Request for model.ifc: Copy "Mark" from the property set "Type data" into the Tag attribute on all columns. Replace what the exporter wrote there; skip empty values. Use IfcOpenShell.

First a look at what the model holds.

```python
import ifcopenshell
import ifcopenshell.util.element

model = ifcopenshell.open("model.ifc")
print(model.schema)
columns = model.by_type("IfcColumn")
print(len(columns), "columns")
for e in columns[:8]:
    source = ifcopenshell.util.element.get_pset(e, "Type data", "Mark")
    target = e.Tag
    print(e.id(), repr(source), repr(target), sep=" | ")
```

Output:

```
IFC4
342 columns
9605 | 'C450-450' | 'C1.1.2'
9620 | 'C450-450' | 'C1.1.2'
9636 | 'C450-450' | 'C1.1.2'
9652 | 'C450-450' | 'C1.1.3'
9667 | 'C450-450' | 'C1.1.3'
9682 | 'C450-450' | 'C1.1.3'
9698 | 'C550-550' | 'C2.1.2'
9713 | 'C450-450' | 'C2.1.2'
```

```python
import ifcopenshell
import ifcopenshell.util.element

model = ifcopenshell.open("model.ifc")

count = 0
for e in model.by_type("IfcColumn"):
    value = ifcopenshell.util.element.get_pset(e, "Type data", "Mark")
    current = e.Tag
    if not value or not value.strip() or current == value:
        continue
    e.Tag = value
    count += 1

print(count, "columns updated")

model.write("model_edited.ifc")
```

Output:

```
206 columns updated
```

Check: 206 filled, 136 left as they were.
